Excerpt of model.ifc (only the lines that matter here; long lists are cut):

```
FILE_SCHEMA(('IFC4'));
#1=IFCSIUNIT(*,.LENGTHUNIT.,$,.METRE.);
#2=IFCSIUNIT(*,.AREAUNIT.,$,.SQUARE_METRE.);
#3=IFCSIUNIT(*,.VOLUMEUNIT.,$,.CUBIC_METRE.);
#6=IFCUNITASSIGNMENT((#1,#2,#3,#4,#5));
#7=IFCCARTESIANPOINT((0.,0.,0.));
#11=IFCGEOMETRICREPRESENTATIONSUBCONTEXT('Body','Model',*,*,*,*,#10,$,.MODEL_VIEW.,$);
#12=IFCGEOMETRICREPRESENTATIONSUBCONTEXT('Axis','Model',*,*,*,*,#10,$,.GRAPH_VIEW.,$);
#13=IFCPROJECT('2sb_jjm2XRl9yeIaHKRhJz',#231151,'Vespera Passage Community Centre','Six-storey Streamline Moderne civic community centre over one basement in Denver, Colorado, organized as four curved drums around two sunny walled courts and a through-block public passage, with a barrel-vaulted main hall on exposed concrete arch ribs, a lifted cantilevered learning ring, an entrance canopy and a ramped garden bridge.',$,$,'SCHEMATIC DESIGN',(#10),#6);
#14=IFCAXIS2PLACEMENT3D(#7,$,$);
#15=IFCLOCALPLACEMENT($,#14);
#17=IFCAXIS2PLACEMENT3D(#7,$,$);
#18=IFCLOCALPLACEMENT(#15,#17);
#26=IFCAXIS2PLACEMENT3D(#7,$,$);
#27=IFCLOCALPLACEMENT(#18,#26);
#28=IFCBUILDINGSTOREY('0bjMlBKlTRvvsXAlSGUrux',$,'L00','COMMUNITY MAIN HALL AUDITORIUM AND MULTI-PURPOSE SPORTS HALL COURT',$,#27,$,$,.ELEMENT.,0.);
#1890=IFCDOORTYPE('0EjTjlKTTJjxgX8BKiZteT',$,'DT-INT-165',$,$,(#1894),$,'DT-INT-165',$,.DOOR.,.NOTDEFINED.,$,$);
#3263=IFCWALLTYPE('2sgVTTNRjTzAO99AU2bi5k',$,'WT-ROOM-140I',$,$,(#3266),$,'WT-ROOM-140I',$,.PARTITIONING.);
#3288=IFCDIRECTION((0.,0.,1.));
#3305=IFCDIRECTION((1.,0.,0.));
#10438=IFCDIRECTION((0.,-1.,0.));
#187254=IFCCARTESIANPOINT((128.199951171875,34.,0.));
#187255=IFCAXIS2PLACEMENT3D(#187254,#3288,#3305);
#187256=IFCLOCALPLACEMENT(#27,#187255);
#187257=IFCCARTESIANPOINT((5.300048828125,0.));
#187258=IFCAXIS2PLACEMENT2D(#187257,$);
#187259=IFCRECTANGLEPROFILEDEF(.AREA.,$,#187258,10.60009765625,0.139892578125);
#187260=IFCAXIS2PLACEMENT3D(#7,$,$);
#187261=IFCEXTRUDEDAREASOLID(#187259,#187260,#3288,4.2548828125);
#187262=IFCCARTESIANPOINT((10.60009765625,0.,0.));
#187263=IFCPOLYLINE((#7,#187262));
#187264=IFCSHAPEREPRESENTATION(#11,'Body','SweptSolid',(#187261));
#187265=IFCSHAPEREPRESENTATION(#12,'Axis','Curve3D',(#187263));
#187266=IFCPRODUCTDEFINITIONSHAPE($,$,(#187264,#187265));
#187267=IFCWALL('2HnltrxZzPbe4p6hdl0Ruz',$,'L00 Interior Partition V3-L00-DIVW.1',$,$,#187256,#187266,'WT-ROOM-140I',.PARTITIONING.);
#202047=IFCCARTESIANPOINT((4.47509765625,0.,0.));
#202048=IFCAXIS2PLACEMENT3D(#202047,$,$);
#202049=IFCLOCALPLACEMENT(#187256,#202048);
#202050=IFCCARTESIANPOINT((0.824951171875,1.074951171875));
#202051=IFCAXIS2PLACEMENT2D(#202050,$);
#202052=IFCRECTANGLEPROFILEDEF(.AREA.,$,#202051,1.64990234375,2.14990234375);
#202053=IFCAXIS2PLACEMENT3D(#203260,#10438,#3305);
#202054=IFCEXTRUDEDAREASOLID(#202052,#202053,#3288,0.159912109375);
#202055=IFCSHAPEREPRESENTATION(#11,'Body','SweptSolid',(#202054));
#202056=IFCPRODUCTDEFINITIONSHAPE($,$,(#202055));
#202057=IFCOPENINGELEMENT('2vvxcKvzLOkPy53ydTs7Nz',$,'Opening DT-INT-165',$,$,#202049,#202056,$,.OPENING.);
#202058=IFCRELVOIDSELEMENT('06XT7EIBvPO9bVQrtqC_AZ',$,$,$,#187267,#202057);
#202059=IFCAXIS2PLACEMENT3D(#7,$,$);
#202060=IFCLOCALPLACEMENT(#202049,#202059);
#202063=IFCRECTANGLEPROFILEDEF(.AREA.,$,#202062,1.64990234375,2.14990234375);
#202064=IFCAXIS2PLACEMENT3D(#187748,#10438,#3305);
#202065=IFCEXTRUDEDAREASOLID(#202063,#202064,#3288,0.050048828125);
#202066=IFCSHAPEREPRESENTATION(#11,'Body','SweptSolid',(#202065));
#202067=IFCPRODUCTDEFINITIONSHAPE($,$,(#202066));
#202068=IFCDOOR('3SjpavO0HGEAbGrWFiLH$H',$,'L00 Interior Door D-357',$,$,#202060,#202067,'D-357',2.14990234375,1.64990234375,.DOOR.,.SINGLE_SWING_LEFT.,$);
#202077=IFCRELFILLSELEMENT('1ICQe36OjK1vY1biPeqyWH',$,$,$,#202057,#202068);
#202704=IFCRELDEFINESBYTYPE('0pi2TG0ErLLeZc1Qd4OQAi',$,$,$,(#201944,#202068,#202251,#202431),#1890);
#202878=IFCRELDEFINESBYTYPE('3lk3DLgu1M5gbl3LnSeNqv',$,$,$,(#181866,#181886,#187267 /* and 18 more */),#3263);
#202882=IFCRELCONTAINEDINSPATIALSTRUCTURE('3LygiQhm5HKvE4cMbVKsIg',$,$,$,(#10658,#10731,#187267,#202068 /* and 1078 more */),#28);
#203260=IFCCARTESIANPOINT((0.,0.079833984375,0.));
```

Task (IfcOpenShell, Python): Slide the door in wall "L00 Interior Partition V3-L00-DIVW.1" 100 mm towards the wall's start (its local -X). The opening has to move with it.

```python
import ifcopenshell
import ifcopenshell.api.geometry
import ifcopenshell.util.placement

model = ifcopenshell.open("model.ifc")

door = model.by_guid("3SjpavO0HGEAbGrWFiLH$H")
opening = door.FillsVoids[0].RelatingOpeningElement
wall = opening.VoidsElements[0].RelatingBuildingElement

wall_matrix = ifcopenshell.util.placement.get_local_placement(wall.ObjectPlacement)
shift = wall_matrix[:3, 0] * -0.1
before = ifcopenshell.util.placement.get_local_placement(door.ObjectPlacement)[:3, 3].copy()

# The door is placed relative to its opening, so it follows when the opening moves.
matrix = ifcopenshell.util.placement.get_local_placement(opening.ObjectPlacement)
matrix[:3, 3] += shift
ifcopenshell.api.geometry.edit_object_placement(
    model, product=opening, matrix=matrix, is_si=False, should_transform_children=True
)

after = ifcopenshell.util.placement.get_local_placement(door.ObjectPlacement)[:3, 3]
print("door moved by", (after - before).round(3) + 0.0)

model.write("model-out.ifc")
```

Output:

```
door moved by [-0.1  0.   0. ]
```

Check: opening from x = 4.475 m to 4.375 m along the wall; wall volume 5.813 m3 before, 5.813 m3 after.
